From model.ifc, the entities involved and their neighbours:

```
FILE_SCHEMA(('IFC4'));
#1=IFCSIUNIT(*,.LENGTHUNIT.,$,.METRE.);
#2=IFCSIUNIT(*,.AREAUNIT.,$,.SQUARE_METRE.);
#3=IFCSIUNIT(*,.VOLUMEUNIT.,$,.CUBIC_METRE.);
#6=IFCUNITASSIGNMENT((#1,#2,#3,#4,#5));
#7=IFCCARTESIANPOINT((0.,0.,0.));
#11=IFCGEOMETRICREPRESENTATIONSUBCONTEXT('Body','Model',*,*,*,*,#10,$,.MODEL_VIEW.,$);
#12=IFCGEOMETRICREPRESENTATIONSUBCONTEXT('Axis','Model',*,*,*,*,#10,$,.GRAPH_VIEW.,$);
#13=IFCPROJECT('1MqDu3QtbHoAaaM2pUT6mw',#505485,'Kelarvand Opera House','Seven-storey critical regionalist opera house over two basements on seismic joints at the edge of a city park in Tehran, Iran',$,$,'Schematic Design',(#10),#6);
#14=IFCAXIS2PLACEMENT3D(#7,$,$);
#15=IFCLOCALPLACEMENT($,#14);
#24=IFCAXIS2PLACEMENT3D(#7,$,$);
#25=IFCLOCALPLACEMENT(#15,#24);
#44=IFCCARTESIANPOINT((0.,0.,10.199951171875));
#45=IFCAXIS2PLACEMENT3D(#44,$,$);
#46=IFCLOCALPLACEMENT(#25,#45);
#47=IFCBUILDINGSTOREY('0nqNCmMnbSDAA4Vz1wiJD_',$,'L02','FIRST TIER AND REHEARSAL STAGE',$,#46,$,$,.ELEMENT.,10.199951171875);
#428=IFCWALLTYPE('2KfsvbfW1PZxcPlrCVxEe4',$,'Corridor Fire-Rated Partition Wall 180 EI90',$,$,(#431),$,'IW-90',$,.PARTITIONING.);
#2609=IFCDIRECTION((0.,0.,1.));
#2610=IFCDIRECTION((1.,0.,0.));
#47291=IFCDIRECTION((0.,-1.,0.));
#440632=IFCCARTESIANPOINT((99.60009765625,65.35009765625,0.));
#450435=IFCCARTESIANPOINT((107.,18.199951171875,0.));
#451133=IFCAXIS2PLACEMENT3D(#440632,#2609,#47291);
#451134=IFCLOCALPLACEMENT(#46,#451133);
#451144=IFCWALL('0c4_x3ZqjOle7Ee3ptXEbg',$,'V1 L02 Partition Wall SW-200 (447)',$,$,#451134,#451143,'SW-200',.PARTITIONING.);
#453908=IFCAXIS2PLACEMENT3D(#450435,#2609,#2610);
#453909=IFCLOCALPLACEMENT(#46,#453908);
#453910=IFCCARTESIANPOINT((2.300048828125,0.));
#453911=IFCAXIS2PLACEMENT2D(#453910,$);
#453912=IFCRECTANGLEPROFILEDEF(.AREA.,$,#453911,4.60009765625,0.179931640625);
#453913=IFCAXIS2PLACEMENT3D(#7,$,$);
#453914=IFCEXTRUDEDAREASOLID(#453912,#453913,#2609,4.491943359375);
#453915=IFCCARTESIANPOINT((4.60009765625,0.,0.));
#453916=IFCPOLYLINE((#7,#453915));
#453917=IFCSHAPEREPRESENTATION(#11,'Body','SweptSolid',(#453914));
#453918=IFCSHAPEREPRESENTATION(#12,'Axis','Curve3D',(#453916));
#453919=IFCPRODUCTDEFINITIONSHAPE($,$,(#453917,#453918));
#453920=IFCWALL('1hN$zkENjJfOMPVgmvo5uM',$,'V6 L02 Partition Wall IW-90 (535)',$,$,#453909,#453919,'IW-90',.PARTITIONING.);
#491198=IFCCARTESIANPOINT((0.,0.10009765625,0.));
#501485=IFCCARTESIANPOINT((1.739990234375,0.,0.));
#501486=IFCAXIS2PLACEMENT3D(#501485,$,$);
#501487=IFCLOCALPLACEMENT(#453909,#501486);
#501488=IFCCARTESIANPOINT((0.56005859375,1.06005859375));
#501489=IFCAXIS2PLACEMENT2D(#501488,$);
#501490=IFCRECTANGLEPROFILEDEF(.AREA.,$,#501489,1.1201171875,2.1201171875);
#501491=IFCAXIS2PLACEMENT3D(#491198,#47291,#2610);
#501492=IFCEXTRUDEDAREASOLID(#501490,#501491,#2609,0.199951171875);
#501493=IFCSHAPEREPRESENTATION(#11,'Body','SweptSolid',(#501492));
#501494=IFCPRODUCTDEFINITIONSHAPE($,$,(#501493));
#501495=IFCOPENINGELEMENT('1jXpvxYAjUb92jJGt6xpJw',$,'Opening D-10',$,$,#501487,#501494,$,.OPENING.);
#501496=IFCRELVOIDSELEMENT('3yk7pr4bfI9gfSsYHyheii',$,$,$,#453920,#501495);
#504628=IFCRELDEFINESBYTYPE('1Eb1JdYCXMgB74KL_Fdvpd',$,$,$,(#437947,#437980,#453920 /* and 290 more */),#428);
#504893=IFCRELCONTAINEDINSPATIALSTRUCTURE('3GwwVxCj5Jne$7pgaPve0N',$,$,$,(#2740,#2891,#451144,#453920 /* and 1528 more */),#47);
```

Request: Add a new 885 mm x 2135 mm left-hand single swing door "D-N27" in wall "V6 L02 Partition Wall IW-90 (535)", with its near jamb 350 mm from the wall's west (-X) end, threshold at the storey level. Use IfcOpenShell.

```python
import numpy as np
import ifcopenshell
import ifcopenshell.api.feature
import ifcopenshell.api.geometry
import ifcopenshell.api.root
import ifcopenshell.api.spatial
import ifcopenshell.geom
import ifcopenshell.util.element
import ifcopenshell.util.placement
import ifcopenshell.util.representation
import ifcopenshell.util.shape
import ifcopenshell.util.unit

model = ifcopenshell.open("model.ifc")
unit_scale = ifcopenshell.util.unit.calculate_unit_scale(model)
settings = ifcopenshell.geom.settings()


def volume(element):
    """Net volume in cubic metres, openings subtracted."""
    shape = ifcopenshell.geom.create_shape(settings, element)
    return ifcopenshell.util.shape.get_volume(shape.geometry)


wall = model.by_guid("1hN$zkENjJfOMPVgmvo5uM")
storey = ifcopenshell.util.element.get_container(wall, ifc_class="IfcBuildingStorey")
context = ifcopenshell.util.representation.get_context(model, "Model", "Body", "MODEL_VIEW")
before = volume(wall)

width, height, from_end, sill = 0.885, 2.135, 0.35, 0.0  # metres

# The wall runs along its own X axis, and the end named is its -X end.
wall_shape = ifcopenshell.geom.create_shape(settings, wall)
x, y, z = ifcopenshell.util.shape.get_vertices(wall_shape.geometry).T
start = x.min() + from_end
face, thickness = float(y.min()), float(y.max() - y.min())
wall_matrix = ifcopenshell.util.placement.get_local_placement(wall.ObjectPlacement)
level = ifcopenshell.util.placement.get_local_placement(storey.ObjectPlacement)[2, 3]


def in_wall(x, y):
    """Placement at x, y metres in the wall's axes, at sill height."""
    matrix = wall_matrix.copy()
    matrix[:, 3] = wall_matrix @ np.array([x / unit_scale, y / unit_scale, 0.0, 1.0])
    matrix[2, 3] = level + sill / unit_scale
    return matrix


# Opening: a box that overshoots both wall faces by 50 mm.
opening = ifcopenshell.api.root.create_entity(model, ifc_class="IfcOpeningElement", predefined_type="OPENING")
box = ifcopenshell.api.geometry.add_wall_representation(
    model, context=context, length=width, height=height, thickness=thickness + 0.1
)
ifcopenshell.api.geometry.assign_representation(model, product=opening, representation=box)
ifcopenshell.api.geometry.edit_object_placement(model, product=opening, matrix=in_wall(start, face - 0.05), is_si=False)
ifcopenshell.api.feature.add_feature(model, feature=opening, element=wall)

door = ifcopenshell.api.root.create_entity(model, ifc_class="IfcDoor", name="D-N27", predefined_type="DOOR")
door.OverallWidth, door.OverallHeight = width / unit_scale, height / unit_scale
door.OperationType = "SINGLE_SWING_LEFT"
body = ifcopenshell.api.geometry.add_door_representation(
    model,
    context=context,
    overall_width=door.OverallWidth,
    overall_height=door.OverallHeight,
    operation_type="SINGLE_SWING_LEFT",
    lining_properties={"LiningDepth": thickness / unit_scale, "ThresholdDepth": thickness / unit_scale},
)
ifcopenshell.api.geometry.assign_representation(model, product=door, representation=body)
ifcopenshell.api.spatial.assign_container(model, products=[door], relating_structure=storey)
ifcopenshell.api.feature.add_filling(model, opening=opening, element=door)

# The lining spans the wall, so the door starts at the wall face.
ifcopenshell.api.geometry.edit_object_placement(model, product=door, matrix=in_wall(start, face), is_si=False)

after = volume(wall)

print(f"wall volume {before:.3f} -> {after:.3f} m3")

model.write("model_rev.ifc")
```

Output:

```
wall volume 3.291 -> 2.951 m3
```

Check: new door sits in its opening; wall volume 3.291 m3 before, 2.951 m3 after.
